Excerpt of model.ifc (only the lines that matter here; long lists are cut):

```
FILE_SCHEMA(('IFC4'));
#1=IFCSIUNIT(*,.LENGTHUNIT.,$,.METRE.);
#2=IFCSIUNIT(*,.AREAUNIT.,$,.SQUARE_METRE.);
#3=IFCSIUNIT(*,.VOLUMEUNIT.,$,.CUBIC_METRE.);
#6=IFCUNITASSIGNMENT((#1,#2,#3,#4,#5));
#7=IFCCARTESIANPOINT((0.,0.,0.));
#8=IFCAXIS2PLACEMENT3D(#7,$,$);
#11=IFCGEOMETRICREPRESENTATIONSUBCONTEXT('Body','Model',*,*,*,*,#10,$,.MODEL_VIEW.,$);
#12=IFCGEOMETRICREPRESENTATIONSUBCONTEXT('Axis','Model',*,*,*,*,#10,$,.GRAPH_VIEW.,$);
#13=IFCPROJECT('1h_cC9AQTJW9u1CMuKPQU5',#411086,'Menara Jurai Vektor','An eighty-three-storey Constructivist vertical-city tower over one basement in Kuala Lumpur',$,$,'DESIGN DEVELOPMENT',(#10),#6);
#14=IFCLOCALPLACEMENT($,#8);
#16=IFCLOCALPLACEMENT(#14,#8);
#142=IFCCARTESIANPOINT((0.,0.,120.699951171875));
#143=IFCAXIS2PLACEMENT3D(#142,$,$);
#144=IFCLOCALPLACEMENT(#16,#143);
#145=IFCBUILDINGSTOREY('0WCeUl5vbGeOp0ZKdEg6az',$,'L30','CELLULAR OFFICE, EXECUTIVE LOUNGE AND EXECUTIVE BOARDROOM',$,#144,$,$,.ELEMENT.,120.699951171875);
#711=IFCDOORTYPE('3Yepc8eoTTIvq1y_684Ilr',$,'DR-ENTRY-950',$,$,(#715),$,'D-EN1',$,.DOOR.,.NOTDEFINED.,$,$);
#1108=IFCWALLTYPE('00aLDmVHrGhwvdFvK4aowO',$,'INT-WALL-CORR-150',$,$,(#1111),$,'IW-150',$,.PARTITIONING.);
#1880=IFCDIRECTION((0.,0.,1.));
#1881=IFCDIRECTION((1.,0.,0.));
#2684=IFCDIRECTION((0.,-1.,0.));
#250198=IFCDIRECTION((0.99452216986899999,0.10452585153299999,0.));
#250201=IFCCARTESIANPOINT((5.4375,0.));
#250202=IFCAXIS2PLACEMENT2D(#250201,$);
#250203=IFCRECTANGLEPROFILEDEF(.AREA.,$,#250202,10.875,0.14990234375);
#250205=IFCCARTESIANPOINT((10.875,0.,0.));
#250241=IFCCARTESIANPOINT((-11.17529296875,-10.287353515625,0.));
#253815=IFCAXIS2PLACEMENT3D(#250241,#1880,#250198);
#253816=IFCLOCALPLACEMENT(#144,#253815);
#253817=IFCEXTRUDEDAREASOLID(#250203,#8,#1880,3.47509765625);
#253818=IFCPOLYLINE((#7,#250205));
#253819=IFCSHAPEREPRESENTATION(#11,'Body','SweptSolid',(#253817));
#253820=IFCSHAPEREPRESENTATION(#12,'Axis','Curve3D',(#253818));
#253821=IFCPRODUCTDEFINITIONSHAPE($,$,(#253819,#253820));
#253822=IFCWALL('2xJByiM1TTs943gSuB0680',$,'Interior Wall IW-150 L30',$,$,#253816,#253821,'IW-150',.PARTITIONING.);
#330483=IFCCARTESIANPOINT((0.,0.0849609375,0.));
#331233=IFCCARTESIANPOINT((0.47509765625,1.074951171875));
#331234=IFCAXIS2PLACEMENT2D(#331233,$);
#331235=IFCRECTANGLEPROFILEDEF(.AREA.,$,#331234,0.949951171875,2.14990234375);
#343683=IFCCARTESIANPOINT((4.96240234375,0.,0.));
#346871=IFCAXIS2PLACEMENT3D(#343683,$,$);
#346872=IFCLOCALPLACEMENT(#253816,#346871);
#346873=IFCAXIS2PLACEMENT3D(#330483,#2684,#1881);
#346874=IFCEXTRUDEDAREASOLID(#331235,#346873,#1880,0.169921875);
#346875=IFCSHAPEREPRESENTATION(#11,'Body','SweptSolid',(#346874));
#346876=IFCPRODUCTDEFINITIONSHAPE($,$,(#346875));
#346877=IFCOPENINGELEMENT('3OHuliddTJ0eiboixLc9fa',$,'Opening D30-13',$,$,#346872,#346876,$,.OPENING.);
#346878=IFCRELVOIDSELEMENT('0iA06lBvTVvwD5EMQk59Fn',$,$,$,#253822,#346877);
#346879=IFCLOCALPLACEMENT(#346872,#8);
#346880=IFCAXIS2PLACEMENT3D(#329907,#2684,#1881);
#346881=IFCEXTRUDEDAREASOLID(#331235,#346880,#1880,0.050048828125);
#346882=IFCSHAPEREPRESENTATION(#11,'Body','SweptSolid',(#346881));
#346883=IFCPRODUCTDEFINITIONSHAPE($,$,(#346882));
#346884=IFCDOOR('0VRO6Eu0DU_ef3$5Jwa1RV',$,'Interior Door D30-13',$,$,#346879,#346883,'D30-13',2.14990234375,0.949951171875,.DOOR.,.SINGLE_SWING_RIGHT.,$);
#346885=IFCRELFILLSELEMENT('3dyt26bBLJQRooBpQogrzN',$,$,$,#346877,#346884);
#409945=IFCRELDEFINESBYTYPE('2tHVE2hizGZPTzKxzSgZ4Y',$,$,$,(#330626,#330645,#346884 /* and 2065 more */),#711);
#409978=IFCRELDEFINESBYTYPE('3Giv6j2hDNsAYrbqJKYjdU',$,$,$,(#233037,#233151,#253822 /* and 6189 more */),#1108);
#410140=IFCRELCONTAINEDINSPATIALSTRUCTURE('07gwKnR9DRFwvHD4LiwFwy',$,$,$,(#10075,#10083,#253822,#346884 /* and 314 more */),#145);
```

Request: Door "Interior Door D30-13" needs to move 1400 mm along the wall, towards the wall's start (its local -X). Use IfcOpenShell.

```python
import ifcopenshell
import ifcopenshell.api.geometry
import ifcopenshell.util.placement
import ifcopenshell.util.unit

model = ifcopenshell.open("model.ifc")
unit_scale = ifcopenshell.util.unit.calculate_unit_scale(model)

door = model.by_guid("0VRO6Eu0DU_ef3$5Jwa1RV")
opening = door.FillsVoids[0].RelatingOpeningElement
wall = opening.VoidsElements[0].RelatingBuildingElement

wall_matrix = ifcopenshell.util.placement.get_local_placement(wall.ObjectPlacement)
shift = wall_matrix[:3, 0] * -1.4 / unit_scale
before = ifcopenshell.util.placement.get_local_placement(door.ObjectPlacement)[:3, 3].copy()

# The door is placed relative to its opening, so it follows when the opening moves.
matrix = ifcopenshell.util.placement.get_local_placement(opening.ObjectPlacement)
matrix[:3, 3] += shift
ifcopenshell.api.geometry.edit_object_placement(
    model, product=opening, matrix=matrix, is_si=False, should_transform_children=True
)

after = ifcopenshell.util.placement.get_local_placement(door.ObjectPlacement)[:3, 3]
print("door moved by", (after - before).round(3) + 0.0)

model.write("model_updated.ifc")
```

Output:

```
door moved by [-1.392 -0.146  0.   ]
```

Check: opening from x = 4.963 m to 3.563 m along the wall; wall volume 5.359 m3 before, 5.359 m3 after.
